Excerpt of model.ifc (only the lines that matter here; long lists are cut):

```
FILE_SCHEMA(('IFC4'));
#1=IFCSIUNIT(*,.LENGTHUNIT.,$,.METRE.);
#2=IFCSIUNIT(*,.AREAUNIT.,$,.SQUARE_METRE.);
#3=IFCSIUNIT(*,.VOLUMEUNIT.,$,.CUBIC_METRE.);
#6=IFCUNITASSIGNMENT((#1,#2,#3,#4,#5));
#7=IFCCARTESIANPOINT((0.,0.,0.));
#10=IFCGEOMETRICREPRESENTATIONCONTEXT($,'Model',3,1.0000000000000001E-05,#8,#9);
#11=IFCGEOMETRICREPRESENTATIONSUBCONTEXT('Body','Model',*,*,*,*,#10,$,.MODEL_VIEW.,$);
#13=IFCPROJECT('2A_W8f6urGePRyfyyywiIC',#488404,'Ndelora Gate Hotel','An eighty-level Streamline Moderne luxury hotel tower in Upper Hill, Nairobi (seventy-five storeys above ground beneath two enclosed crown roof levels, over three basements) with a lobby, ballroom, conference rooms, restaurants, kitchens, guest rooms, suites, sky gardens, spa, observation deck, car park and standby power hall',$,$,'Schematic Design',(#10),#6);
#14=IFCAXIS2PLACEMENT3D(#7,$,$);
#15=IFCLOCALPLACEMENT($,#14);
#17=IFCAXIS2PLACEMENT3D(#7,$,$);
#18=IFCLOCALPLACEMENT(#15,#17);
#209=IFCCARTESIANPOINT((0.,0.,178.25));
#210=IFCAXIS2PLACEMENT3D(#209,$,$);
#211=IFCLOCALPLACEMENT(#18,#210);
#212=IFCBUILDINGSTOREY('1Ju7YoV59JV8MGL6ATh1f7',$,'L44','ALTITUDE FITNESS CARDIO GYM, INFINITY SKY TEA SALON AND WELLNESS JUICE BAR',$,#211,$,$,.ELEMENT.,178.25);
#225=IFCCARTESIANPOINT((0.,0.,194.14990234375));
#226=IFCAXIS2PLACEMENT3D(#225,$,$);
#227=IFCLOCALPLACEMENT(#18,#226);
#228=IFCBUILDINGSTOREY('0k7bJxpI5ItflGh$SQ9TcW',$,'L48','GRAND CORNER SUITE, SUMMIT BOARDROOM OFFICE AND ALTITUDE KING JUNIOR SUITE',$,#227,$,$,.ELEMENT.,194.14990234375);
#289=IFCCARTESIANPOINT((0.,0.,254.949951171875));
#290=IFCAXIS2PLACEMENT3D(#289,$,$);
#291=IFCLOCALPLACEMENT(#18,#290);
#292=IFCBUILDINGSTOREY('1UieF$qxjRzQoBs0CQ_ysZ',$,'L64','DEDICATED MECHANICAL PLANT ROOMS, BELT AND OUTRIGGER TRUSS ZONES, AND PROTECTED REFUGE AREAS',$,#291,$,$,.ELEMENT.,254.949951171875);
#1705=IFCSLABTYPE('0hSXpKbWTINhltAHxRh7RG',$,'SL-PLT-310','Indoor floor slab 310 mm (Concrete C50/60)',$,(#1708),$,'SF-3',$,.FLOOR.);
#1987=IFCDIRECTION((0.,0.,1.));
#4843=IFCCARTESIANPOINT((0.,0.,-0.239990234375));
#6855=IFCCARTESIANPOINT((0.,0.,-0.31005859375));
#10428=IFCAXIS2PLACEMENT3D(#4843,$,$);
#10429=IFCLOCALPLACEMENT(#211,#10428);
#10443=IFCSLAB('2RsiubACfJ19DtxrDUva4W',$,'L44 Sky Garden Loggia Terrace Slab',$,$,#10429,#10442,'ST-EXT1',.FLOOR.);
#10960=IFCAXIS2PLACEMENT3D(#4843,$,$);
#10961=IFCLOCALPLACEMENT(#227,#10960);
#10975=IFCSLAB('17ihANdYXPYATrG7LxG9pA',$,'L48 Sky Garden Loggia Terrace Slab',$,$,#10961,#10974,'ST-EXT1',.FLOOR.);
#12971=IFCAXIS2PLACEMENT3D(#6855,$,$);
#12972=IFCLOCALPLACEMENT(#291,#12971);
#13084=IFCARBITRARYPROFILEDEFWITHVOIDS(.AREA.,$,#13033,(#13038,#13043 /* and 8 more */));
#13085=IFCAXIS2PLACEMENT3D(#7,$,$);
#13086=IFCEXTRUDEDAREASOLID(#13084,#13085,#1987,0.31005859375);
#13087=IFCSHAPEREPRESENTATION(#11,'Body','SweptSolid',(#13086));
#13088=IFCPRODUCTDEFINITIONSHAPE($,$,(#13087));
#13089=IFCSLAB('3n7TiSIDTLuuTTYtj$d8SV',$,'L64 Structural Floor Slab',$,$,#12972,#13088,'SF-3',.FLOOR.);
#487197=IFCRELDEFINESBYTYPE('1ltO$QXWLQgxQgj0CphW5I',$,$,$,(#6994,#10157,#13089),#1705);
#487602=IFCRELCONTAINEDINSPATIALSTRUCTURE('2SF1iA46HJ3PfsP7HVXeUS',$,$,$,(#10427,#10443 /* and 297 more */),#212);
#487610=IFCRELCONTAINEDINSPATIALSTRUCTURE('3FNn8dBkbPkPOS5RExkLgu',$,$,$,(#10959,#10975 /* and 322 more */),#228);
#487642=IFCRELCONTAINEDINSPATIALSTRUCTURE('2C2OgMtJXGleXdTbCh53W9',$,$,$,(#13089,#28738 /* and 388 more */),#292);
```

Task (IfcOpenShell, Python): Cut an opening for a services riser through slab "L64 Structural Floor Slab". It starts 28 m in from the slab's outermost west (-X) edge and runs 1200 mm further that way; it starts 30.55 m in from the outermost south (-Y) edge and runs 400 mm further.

```python
import numpy as np
import ifcopenshell
import ifcopenshell.api.feature
import ifcopenshell.api.geometry
import ifcopenshell.api.root
import ifcopenshell.geom
import ifcopenshell.util.placement
import ifcopenshell.util.representation
import ifcopenshell.util.shape
import ifcopenshell.util.unit

model = ifcopenshell.open("model.ifc")
unit_scale = ifcopenshell.util.unit.calculate_unit_scale(model)
settings = ifcopenshell.geom.settings()


def volume(element):
    """Net volume in cubic metres, openings subtracted."""
    shape = ifcopenshell.geom.create_shape(settings, element)
    return ifcopenshell.util.shape.get_volume(shape.geometry)


slab = model.by_guid("3n7TiSIDTLuuTTYtj$d8SV")
before = volume(slab)

# Extent in the slab's own axes, in metres. The edges named are its -X and -Y sides.
slab_shape = ifcopenshell.geom.create_shape(settings, slab)
vertices = ifcopenshell.util.shape.get_vertices(slab_shape.geometry)
x_min, y_min, bottom = vertices.min(axis=0)
top = vertices[:, 2].max()

opening = ifcopenshell.api.root.create_entity(model, ifc_class="IfcOpeningElement", name="Services riser opening", predefined_type="OPENING")
context = ifcopenshell.util.representation.get_context(model, "Model", "Body", "MODEL_VIEW")
width, depth = 1.2, 0.4
outline = [(0.0, 0.0), (width, 0.0), (width, depth), (0.0, depth), (0.0, 0.0)]
# Overshoot both faces by 50 mm so the cut is clean.
shape = ifcopenshell.api.geometry.add_slab_representation(
    model, context=context, depth=top - bottom + 0.1, polyline=outline
)
ifcopenshell.api.geometry.assign_representation(model, product=opening, representation=shape)

matrix = ifcopenshell.util.placement.get_local_placement(slab.ObjectPlacement)
matrix[:, 3] = matrix @ np.append(np.array([x_min + 28, y_min + 30.55, bottom - 0.05]) / unit_scale, 1.0)
ifcopenshell.api.geometry.edit_object_placement(model, product=opening, matrix=matrix, is_si=False)
ifcopenshell.api.feature.add_feature(model, feature=opening, element=slab)

after = volume(slab)

print(f"slab volume {before:.3f} -> {after:.3f} m3")

model.write("model-out.ifc")
```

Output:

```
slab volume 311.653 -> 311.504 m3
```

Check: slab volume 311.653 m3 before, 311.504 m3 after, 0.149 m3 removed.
